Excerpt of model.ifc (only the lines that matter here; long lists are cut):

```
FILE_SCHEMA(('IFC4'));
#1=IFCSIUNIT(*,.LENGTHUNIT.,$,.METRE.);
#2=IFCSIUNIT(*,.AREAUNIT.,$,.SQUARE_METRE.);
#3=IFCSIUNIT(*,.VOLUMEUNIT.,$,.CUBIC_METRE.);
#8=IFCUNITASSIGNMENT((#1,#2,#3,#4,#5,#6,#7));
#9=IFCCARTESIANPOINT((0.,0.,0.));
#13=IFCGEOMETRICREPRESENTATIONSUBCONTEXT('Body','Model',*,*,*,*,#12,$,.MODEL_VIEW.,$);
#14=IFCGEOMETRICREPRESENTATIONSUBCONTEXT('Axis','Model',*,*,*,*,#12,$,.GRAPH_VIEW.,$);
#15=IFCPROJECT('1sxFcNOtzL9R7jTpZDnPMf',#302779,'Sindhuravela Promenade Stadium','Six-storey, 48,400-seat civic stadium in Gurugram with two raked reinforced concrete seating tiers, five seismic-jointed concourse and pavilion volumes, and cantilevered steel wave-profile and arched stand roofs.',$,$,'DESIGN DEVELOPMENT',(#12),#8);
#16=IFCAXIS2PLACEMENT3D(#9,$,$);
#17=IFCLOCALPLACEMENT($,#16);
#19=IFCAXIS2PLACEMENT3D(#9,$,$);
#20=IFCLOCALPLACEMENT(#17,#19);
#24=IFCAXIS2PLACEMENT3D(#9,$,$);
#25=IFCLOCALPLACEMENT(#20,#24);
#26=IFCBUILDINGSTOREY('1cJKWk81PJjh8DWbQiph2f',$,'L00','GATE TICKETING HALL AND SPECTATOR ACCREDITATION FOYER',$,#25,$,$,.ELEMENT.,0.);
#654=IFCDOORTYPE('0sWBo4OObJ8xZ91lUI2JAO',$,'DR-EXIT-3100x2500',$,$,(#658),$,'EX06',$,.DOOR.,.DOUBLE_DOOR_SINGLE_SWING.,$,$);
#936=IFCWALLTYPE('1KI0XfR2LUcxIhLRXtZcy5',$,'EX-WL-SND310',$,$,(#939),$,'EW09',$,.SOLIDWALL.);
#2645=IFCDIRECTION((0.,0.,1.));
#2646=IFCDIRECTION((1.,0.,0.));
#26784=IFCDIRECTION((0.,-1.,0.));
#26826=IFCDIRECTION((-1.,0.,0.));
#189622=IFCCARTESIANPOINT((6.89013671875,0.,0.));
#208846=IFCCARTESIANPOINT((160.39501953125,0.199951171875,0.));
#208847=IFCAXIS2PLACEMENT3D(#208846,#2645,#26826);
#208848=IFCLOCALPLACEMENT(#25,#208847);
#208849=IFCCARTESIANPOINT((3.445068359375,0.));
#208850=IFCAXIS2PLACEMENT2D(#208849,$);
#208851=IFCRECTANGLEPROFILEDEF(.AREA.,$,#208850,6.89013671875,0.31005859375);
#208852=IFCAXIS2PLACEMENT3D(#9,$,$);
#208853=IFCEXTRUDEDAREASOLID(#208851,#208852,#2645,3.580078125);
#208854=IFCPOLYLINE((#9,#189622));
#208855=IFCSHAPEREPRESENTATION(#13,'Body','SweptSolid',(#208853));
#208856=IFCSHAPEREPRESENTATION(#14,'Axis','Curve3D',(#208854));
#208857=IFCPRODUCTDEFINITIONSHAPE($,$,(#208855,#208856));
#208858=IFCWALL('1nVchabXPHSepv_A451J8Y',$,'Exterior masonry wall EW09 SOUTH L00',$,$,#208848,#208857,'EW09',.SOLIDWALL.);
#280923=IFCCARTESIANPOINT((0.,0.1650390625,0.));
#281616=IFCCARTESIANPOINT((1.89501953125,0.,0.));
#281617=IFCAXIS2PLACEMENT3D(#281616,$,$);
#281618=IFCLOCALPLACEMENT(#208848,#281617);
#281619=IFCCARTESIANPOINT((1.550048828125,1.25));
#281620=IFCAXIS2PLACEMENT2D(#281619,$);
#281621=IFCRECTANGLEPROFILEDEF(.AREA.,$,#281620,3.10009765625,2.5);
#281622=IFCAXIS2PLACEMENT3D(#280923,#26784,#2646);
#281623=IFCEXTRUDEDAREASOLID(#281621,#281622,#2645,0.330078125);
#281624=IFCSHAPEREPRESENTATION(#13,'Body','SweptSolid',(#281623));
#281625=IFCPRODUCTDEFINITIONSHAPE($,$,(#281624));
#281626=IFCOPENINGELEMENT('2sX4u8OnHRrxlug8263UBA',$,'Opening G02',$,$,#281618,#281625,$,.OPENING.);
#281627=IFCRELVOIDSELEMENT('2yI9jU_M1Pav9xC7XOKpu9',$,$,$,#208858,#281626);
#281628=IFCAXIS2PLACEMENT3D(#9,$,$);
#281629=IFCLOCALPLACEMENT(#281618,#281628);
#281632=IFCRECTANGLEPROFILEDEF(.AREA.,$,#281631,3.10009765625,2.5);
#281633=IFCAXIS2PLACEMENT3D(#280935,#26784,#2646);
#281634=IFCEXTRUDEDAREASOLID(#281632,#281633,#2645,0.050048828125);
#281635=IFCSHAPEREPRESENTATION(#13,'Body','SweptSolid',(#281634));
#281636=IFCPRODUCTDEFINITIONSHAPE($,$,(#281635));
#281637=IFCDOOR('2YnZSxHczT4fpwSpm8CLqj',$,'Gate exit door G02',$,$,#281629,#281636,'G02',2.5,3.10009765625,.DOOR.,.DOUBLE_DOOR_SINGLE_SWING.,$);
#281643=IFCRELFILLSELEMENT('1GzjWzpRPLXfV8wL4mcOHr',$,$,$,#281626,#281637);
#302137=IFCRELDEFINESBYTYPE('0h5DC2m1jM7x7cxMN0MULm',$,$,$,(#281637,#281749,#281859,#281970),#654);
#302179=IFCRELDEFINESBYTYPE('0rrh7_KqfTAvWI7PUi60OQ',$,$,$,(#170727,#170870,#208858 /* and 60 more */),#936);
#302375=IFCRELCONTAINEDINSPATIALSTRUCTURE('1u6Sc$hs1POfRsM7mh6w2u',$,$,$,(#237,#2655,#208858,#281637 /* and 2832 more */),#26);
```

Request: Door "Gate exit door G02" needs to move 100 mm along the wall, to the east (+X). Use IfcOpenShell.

```python
import ifcopenshell
import ifcopenshell.api.geometry
import ifcopenshell.util.placement

model = ifcopenshell.open("model.ifc")

door = model.by_guid("2YnZSxHczT4fpwSpm8CLqj")
opening = door.FillsVoids[0].RelatingOpeningElement
wall = opening.VoidsElements[0].RelatingBuildingElement

wall_matrix = ifcopenshell.util.placement.get_local_placement(wall.ObjectPlacement)
shift = wall_matrix[:3, 0] * -0.1
before = ifcopenshell.util.placement.get_local_placement(door.ObjectPlacement)[:3, 3].copy()

# The door is placed relative to its opening, so it follows when the opening moves.
matrix = ifcopenshell.util.placement.get_local_placement(opening.ObjectPlacement)
matrix[:3, 3] += shift
ifcopenshell.api.geometry.edit_object_placement(
    model, product=opening, matrix=matrix, is_si=False, should_transform_children=True
)

after = ifcopenshell.util.placement.get_local_placement(door.ObjectPlacement)[:3, 3]
print("door moved by", (after - before).round(3) + 0.0)

model.write("model-out.ifc")
```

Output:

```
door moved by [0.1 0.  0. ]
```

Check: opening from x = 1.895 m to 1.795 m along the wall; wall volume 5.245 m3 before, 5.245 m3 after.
